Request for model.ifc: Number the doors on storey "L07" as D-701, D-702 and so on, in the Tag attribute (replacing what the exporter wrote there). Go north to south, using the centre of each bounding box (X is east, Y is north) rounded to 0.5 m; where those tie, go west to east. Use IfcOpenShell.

First a look at what the model holds.

```python
import ifcopenshell
import ifcopenshell.util.element
import ifcopenshell.util.placement

model = ifcopenshell.open("model.ifc")
print(model.schema)
storey = next(s for s in model.by_type("IfcBuildingStorey") if s.Name == "L07")
doors = [e for e in ifcopenshell.util.element.get_decomposition(storey) if e.is_a("IfcDoor")]
for e in sorted(doors, key=lambda e: e.id()):
    origin = ifcopenshell.util.placement.get_local_placement(e.ObjectPlacement)[:3, 3]
    print(e.id(), e.Tag, e.Name, origin.round(2) + 0.0, sep=" | ")
```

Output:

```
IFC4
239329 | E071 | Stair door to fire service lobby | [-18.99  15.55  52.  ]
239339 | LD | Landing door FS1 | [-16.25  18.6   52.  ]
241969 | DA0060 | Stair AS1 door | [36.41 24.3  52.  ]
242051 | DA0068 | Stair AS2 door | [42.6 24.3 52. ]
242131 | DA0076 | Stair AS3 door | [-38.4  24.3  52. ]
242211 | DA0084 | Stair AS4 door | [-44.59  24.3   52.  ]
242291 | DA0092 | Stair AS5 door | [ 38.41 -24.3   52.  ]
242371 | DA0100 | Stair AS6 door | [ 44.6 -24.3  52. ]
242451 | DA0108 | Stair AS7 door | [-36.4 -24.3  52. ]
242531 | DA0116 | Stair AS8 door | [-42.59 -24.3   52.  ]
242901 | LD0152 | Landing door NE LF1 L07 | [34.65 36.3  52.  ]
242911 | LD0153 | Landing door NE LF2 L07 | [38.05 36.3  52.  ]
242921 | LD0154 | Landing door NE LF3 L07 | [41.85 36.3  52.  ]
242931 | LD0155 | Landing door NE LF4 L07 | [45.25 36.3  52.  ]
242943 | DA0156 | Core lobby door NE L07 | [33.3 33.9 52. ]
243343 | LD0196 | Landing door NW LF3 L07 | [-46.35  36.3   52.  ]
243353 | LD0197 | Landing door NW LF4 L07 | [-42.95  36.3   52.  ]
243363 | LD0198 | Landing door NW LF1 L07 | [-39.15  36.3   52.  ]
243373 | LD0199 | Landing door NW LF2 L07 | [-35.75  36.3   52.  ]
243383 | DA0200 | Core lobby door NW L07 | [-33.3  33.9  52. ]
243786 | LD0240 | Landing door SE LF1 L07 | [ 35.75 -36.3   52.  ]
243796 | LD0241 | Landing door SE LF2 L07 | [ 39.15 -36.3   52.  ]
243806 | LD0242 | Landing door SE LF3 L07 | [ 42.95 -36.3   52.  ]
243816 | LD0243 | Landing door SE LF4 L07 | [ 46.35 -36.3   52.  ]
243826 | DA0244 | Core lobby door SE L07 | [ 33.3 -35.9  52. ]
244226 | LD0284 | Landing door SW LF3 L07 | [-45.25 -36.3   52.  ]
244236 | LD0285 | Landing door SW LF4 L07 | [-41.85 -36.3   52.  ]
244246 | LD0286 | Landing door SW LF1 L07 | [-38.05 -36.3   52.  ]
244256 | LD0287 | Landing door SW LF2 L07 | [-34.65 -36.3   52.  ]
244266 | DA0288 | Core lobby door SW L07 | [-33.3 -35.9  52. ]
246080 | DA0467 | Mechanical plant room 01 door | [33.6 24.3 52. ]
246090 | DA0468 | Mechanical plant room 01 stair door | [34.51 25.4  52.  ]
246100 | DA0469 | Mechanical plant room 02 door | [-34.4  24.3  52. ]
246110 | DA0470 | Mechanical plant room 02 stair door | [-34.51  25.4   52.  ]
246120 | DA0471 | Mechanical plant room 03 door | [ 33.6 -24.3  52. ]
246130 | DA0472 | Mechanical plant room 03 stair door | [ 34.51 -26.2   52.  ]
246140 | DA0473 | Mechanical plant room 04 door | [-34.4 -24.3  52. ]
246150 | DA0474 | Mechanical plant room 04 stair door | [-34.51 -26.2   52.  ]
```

```python
import ifcopenshell
import ifcopenshell.geom
import ifcopenshell.util.element
import ifcopenshell.util.shape

model = ifcopenshell.open("model.ifc")
settings = ifcopenshell.geom.settings()
settings.set("use-world-coords", True)


def centre(element):
    shape = ifcopenshell.geom.create_shape(settings, element)
    return ifcopenshell.util.shape.get_bbox_centroid(shape.geometry)


storey = next(s for s in model.by_type("IfcBuildingStorey") if s.Name == "L07")
doors = [e for e in ifcopenshell.util.element.get_decomposition(storey) if e.is_a("IfcDoor")]

# Insertion points can sit at a corner or the storey origin, so sort by the geometry (in metres).
centres = {e: centre(e) for e in doors}
doors.sort(key=lambda e: (-round(centres[e][1] / 0.5), centres[e][0]))

for i, e in enumerate(doors, start=1):
    number = f"D-7{i:02d}"
    e.Tag = number
    print(e.id(), number)

model.write("model-out.ifc")
```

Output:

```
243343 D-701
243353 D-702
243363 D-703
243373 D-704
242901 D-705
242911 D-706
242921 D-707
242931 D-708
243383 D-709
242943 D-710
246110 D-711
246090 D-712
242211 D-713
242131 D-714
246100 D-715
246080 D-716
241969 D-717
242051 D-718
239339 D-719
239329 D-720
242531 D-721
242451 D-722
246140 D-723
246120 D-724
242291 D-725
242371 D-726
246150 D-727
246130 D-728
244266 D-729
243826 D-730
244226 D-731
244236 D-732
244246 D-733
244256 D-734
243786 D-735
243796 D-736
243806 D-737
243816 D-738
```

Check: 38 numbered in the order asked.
